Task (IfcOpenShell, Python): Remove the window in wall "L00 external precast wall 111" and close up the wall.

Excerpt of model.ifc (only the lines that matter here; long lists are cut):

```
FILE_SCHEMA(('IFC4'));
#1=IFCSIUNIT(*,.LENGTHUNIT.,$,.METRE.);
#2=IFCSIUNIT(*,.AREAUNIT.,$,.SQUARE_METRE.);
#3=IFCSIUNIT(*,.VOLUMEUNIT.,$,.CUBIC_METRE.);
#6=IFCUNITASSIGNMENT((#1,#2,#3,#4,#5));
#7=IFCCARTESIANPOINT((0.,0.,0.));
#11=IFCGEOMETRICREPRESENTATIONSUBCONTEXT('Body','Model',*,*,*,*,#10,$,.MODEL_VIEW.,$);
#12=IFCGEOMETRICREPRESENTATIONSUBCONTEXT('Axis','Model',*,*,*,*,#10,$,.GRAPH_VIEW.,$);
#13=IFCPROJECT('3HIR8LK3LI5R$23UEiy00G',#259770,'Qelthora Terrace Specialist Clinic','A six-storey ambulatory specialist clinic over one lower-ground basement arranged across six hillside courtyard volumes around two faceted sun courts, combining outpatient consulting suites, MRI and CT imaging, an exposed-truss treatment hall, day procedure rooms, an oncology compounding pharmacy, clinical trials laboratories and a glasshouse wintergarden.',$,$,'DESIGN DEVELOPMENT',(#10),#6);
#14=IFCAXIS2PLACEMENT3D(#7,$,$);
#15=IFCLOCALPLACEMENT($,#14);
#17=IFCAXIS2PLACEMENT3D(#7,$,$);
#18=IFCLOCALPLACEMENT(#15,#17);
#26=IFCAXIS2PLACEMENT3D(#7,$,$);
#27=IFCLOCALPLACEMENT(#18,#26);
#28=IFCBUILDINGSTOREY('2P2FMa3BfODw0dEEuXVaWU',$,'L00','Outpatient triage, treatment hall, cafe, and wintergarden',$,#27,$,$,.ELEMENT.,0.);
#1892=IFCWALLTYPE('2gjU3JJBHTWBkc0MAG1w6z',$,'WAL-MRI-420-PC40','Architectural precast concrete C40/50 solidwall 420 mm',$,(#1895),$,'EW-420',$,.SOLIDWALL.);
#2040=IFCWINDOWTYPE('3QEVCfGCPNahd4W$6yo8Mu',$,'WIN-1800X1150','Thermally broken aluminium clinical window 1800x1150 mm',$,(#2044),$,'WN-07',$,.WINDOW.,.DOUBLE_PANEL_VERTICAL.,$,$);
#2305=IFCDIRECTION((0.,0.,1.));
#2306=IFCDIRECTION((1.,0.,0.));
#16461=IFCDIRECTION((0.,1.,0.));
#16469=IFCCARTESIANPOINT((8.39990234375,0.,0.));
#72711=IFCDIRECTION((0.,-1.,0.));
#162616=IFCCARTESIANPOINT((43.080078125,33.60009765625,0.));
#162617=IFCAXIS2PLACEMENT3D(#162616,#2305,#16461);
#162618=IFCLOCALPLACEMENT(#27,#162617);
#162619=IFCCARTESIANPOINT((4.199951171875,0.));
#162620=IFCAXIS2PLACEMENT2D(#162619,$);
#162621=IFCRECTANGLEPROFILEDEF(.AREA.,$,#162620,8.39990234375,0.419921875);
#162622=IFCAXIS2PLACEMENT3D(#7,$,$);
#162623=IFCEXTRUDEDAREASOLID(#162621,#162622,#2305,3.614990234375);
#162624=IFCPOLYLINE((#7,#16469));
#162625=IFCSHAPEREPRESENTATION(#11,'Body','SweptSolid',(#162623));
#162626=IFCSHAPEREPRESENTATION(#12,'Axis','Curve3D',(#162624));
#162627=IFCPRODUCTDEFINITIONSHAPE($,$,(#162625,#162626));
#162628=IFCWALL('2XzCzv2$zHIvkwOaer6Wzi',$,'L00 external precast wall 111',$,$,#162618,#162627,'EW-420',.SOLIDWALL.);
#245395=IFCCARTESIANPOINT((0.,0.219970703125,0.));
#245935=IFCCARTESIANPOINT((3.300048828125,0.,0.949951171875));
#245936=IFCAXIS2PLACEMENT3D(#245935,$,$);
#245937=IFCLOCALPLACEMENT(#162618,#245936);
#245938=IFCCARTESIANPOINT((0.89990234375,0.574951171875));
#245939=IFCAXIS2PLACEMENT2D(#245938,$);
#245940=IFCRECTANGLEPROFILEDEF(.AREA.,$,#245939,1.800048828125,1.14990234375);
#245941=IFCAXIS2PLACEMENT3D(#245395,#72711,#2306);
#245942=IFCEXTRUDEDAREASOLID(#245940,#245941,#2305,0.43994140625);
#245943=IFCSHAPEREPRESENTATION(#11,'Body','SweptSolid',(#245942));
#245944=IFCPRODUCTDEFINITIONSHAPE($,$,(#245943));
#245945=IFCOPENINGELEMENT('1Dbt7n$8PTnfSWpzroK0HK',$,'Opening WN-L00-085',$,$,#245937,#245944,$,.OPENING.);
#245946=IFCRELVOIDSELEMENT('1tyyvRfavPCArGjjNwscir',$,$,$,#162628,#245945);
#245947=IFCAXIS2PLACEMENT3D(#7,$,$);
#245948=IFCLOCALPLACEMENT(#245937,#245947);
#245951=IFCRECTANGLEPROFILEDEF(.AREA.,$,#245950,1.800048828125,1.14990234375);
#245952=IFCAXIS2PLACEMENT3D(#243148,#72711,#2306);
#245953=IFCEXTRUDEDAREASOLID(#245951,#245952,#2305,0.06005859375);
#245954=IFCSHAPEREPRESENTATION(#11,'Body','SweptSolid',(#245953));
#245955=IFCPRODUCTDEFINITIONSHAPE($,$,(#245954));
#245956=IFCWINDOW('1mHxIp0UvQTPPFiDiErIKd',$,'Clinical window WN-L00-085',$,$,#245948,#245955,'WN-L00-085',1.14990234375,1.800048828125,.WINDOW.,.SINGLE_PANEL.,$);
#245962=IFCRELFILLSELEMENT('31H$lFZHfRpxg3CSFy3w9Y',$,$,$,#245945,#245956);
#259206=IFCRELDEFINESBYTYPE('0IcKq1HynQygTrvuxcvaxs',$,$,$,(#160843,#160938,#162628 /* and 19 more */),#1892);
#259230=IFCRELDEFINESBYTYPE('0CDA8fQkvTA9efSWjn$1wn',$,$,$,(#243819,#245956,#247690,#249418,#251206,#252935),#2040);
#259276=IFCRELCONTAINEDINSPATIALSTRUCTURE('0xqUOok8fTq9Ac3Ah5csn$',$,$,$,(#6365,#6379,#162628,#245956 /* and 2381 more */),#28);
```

```python
import ifcopenshell
import ifcopenshell.api.feature
import ifcopenshell.api.root
import ifcopenshell.geom
import ifcopenshell.util.shape

model = ifcopenshell.open("model.ifc")
settings = ifcopenshell.geom.settings()


def volume(element):
    """Net volume in cubic metres, openings subtracted."""
    shape = ifcopenshell.geom.create_shape(settings, element)
    return ifcopenshell.util.shape.get_volume(shape.geometry)


window = model.by_guid("1mHxIp0UvQTPPFiDiErIKd")
opening = window.FillsVoids[0].RelatingOpeningElement
wall = opening.VoidsElements[0].RelatingBuildingElement
before = volume(wall)

ifcopenshell.api.root.remove_product(model, product=window)
ifcopenshell.api.feature.remove_feature(model, feature=opening)

after = volume(wall)

print(f"wall volume {before:.3f} -> {after:.3f} m3")

model.write("model_edited.ifc")
```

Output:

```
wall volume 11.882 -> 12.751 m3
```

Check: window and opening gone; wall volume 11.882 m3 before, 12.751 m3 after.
